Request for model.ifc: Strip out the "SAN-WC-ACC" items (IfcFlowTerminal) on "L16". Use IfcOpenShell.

First a look at what the model holds.

```python
import ifcopenshell
import ifcopenshell.util.element

model = ifcopenshell.open("model.ifc")
print(model.schema)
storey = next(s for s in model.by_type("IfcBuildingStorey") if s.Name == "L16")
terminals = [e for e in ifcopenshell.util.element.get_decomposition(storey) if e.is_a("IfcFlowTerminal")]
seen = {}
for e in terminals:
    element_type = ifcopenshell.util.element.get_type(e)
    name = element_type.Name if element_type not in (None, e) else None
    seen[name] = seen.get(name, 0) + 1
for name, count in sorted(seen.items(), key=str):
    print(count, "x", name)
```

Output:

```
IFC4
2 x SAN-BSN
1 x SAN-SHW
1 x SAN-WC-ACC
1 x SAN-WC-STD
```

```python
import ifcopenshell
import ifcopenshell.api.root
import ifcopenshell.util.element

model = ifcopenshell.open("model.ifc")

storey = next(s for s in model.by_type("IfcBuildingStorey") if s.Name == "L16")
terminals = [e for e in ifcopenshell.util.element.get_decomposition(storey) if e.is_a("IfcFlowTerminal")]
targets = [e for e in terminals if (t := ifcopenshell.util.element.get_type(e)) not in (None, e) and t.Name == "SAN-WC-ACC"]

for e in targets:
    ifcopenshell.api.root.remove_product(model, product=e)
print(len(targets), "removed")

model.write("model_edited.ifc")
```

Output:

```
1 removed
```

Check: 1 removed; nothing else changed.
